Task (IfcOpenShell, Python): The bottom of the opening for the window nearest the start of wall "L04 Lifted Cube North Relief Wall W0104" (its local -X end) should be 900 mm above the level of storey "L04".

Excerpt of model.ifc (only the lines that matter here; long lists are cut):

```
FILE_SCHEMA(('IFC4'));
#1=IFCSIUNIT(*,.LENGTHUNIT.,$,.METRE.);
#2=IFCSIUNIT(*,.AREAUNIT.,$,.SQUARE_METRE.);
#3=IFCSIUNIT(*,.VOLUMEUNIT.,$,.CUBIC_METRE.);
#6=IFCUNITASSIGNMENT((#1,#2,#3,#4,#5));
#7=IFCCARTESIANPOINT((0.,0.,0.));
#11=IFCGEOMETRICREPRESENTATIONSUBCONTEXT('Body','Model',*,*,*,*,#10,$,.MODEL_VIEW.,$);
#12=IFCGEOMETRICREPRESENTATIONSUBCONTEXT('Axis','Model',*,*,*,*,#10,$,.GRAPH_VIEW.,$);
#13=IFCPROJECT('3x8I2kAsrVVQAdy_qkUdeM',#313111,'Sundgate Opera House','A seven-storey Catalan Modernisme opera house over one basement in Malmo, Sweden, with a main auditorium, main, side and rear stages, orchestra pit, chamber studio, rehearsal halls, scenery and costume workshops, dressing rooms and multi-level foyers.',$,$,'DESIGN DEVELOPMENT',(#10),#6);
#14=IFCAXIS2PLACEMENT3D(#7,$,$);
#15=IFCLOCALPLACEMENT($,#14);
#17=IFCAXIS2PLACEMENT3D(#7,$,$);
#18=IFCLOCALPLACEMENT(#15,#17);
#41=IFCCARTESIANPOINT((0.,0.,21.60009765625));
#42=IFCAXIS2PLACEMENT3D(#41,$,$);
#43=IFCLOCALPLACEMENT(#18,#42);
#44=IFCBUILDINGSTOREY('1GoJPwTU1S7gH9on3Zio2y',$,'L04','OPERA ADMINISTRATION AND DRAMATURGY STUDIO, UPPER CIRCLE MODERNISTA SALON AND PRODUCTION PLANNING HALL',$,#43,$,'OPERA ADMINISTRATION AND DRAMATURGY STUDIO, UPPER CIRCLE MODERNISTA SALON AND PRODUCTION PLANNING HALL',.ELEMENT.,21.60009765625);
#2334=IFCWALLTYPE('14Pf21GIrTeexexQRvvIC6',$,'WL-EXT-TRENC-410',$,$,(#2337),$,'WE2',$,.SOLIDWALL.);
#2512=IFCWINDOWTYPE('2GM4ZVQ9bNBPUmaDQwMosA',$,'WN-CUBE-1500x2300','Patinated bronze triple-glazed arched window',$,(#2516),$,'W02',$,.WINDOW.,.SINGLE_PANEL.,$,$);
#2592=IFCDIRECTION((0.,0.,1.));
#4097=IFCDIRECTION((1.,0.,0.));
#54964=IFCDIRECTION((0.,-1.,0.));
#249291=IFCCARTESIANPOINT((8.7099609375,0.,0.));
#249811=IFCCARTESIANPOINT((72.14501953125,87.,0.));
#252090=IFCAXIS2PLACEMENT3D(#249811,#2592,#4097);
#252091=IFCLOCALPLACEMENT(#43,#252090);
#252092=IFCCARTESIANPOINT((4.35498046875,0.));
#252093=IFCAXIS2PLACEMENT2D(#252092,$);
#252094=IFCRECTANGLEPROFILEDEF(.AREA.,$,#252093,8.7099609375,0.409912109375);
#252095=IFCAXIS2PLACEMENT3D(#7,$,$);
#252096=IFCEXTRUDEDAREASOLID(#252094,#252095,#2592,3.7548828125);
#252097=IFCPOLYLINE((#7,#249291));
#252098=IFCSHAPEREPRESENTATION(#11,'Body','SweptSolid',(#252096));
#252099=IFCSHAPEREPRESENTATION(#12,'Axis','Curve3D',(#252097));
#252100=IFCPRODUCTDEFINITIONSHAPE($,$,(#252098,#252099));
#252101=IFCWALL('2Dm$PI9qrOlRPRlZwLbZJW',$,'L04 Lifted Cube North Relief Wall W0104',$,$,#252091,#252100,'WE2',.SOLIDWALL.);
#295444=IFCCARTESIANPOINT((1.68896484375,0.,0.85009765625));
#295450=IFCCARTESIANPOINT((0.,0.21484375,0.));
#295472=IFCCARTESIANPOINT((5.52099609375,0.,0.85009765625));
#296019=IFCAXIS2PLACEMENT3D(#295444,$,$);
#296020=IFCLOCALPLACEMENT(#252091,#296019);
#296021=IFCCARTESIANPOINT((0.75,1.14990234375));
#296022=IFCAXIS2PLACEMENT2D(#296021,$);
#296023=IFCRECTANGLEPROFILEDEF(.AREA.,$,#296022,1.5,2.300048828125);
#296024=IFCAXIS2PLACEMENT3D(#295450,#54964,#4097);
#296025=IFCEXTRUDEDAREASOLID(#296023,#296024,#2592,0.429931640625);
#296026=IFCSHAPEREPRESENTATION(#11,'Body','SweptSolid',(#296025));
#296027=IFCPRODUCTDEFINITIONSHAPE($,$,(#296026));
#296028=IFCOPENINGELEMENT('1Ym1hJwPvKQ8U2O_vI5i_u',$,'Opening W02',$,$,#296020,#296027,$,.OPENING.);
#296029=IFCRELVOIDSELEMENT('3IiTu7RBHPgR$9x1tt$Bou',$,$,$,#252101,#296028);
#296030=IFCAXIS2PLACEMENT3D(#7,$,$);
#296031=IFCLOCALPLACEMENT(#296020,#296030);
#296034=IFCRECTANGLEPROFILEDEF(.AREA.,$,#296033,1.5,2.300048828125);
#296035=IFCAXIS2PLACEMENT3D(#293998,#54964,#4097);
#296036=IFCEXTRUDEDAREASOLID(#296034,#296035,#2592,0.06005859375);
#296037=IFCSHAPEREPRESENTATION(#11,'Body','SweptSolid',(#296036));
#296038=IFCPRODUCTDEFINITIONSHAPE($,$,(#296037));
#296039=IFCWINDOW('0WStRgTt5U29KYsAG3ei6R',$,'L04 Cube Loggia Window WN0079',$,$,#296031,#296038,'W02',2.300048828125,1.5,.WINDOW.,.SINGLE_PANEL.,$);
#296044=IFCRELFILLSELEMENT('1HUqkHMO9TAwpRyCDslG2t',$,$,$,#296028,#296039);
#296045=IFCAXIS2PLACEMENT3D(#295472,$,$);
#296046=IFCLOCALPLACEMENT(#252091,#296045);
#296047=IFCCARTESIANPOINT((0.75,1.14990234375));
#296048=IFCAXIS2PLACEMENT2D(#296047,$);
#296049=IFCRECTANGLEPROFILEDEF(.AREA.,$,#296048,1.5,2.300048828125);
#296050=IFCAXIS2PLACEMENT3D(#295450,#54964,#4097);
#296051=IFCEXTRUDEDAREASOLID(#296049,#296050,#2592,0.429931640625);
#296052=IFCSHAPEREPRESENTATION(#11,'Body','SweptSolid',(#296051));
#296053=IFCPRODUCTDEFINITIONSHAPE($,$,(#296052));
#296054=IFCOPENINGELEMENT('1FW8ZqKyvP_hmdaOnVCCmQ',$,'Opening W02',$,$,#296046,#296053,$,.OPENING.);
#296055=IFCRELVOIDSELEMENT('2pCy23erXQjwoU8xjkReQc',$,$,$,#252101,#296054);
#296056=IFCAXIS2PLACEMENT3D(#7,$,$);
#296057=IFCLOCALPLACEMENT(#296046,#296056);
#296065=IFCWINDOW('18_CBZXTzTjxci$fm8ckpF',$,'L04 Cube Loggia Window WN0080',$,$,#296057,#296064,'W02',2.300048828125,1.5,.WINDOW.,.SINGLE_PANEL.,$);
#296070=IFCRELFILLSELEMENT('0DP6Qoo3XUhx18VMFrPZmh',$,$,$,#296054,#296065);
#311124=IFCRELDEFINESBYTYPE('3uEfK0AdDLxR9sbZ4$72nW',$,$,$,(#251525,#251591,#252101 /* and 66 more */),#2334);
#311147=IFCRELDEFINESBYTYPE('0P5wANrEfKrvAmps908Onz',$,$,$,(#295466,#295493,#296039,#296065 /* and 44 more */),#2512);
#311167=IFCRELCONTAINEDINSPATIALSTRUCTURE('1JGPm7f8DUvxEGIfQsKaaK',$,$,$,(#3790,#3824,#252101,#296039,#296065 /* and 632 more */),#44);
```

```python
import numpy as np
import ifcopenshell
import ifcopenshell.api.geometry
import ifcopenshell.geom
import ifcopenshell.util.element
import ifcopenshell.util.placement
import ifcopenshell.util.shape
import ifcopenshell.util.unit

model = ifcopenshell.open("model.ifc")
unit_scale = ifcopenshell.util.unit.calculate_unit_scale(model)

window = model.by_guid("0WStRgTt5U29KYsAG3ei6R")
opening = window.FillsVoids[0].RelatingOpeningElement
storey = ifcopenshell.util.element.get_container(window, ifc_class="IfcBuildingStorey")
level = ifcopenshell.util.placement.get_local_placement(storey.ObjectPlacement)[2, 3]

# The opening's origin need not be at the sill, so measure its lowest point.
shape = ifcopenshell.geom.create_shape(ifcopenshell.geom.settings(), opening)
bottom = ifcopenshell.util.shape.get_shape_bottom_elevation(shape, shape.geometry) / unit_scale
dz = level + 0.9 - bottom

shift = np.array([0.0, 0.0, dz])
# The window is placed relative to its opening, so it follows when the opening moves.
matrix = ifcopenshell.util.placement.get_local_placement(opening.ObjectPlacement)
matrix[:3, 3] += shift
ifcopenshell.api.geometry.edit_object_placement(
    model, product=opening, matrix=matrix, is_si=False, should_transform_children=True
)

print(f"moved by {dz * unit_scale:+.3f} m")

model.write("model_v2.ifc")
```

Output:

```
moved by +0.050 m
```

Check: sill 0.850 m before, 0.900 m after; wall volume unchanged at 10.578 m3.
